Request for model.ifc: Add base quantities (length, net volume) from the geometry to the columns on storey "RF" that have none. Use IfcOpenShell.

First a look at what the model holds.

```python
import ifcopenshell
import ifcopenshell.util.element
import ifcopenshell.util.unit

model = ifcopenshell.open("model.ifc")
print(model.schema)
for unit_type in ("LENGTHUNIT", "AREAUNIT", "VOLUMEUNIT"):
    print(unit_type, ifcopenshell.util.unit.calculate_unit_scale(model, unit_type))
storey = next(s for s in model.by_type("IfcBuildingStorey") if s.Name == "RF")
columns = [e for e in ifcopenshell.util.element.get_decomposition(storey) if e.is_a("IfcColumn")]
for e in sorted(columns, key=lambda e: e.id()):
    print(e.id(), e.is_a(), e.Name, list(ifcopenshell.util.element.get_psets(e, qtos_only=True)), sep=" | ")
```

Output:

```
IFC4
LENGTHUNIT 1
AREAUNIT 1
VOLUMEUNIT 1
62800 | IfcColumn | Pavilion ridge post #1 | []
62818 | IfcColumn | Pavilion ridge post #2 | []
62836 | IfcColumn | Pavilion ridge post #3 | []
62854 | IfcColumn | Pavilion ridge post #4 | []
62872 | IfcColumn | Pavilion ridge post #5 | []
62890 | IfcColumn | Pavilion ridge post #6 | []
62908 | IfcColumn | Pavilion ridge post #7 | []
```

```python
import ifcopenshell
import ifcopenshell.api.pset
import ifcopenshell.geom
import ifcopenshell.util.element
import ifcopenshell.util.shape
import ifcopenshell.util.unit

model = ifcopenshell.open("model.ifc")
unit_scale = ifcopenshell.util.unit.calculate_unit_scale(model)
volume_scale = ifcopenshell.util.unit.calculate_unit_scale(model, "VOLUMEUNIT")
settings = ifcopenshell.geom.settings()

storey = next(s for s in model.by_type("IfcBuildingStorey") if s.Name == "RF")
columns = [e for e in ifcopenshell.util.element.get_decomposition(storey) if e.is_a("IfcColumn")]

for e in sorted(columns, key=lambda e: e.id()):
    if ifcopenshell.util.element.get_psets(e, qtos_only=True, should_inherit=False):
        continue
    # Geometry comes back in metres, in the element's own axes.
    shape = ifcopenshell.geom.create_shape(settings, e)
    values = {
        "Length": ifcopenshell.util.shape.get_z(shape.geometry) / unit_scale,
        "NetVolume": ifcopenshell.util.shape.get_volume(shape.geometry) / volume_scale,
    }
    qto = ifcopenshell.api.pset.add_qto(model, product=e, name="Qto_ColumnBaseQuantities")
    ifcopenshell.api.pset.edit_qto(model, qto=qto, properties=values)
    print(e.id(), {k: round(v, 3) for k, v in values.items()})

model.write("model_edited.ifc")
```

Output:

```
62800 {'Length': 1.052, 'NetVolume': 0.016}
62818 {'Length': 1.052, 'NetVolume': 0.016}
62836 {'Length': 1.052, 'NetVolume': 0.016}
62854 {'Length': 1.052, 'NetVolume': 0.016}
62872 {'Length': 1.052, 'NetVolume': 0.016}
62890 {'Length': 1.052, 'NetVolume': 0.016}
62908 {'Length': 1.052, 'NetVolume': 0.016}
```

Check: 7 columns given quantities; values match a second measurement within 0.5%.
